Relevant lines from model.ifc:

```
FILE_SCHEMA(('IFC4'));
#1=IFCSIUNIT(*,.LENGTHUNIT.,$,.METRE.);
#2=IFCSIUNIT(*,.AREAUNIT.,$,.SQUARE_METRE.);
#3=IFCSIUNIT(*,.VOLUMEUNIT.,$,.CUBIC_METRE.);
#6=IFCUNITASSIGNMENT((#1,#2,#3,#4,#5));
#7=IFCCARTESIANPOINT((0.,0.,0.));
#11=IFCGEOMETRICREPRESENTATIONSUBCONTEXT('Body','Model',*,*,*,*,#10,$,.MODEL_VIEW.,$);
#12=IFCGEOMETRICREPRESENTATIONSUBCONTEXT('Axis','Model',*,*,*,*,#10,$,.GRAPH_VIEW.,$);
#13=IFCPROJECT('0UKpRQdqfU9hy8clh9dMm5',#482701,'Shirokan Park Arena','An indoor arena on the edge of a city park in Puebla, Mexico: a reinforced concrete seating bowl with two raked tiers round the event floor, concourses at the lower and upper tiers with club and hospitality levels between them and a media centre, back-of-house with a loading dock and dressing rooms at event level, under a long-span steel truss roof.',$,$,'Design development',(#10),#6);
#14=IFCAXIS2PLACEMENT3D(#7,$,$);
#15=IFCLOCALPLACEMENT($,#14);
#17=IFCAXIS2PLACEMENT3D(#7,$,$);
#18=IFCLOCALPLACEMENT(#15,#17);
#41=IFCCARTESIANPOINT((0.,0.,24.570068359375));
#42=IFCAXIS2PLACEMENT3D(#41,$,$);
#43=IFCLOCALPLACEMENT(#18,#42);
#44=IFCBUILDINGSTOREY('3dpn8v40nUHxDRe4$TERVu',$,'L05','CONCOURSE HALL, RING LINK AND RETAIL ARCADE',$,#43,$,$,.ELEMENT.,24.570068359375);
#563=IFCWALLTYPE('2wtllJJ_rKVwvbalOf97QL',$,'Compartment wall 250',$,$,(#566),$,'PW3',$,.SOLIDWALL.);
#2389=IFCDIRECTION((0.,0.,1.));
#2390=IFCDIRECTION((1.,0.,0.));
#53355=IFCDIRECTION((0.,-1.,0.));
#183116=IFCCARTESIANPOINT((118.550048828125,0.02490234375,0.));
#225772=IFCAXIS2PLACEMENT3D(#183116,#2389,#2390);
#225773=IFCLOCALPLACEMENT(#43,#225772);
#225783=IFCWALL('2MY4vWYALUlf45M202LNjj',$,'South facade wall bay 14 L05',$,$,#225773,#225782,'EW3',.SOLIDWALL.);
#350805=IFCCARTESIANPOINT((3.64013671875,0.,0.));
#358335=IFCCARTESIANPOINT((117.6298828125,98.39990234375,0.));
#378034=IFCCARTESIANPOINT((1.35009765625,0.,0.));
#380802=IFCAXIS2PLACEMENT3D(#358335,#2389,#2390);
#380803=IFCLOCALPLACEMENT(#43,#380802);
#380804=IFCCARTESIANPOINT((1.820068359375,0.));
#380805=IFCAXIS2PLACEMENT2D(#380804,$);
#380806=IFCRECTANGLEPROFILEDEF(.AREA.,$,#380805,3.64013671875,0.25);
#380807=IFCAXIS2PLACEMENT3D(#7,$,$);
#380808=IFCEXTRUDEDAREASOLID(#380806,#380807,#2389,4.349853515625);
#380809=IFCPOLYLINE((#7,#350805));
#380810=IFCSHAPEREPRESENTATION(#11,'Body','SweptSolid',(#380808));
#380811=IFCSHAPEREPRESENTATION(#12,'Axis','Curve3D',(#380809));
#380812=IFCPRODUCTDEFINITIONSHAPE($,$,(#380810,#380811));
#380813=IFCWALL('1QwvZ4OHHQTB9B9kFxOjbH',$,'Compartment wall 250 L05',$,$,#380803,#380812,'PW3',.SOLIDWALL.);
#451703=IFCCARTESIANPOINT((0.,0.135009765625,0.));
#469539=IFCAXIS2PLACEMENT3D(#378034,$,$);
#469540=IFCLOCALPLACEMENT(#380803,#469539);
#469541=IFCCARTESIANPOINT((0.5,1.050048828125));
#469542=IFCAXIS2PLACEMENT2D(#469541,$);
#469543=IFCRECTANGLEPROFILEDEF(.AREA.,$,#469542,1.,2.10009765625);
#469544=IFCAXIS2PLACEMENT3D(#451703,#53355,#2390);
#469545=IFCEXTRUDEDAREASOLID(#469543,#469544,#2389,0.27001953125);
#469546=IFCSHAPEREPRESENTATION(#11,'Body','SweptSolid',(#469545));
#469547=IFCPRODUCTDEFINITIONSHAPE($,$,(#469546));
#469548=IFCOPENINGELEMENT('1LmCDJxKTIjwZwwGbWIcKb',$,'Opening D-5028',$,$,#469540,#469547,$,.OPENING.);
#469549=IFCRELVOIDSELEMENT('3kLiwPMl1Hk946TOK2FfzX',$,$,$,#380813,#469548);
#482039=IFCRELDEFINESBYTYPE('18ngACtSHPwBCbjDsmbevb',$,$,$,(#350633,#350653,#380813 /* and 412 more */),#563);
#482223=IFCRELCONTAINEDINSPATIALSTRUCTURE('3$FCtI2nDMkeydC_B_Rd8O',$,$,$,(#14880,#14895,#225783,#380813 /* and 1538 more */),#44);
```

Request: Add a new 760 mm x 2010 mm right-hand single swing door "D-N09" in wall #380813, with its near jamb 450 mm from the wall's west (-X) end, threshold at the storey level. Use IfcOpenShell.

```python
import numpy as np
import ifcopenshell
import ifcopenshell.api.feature
import ifcopenshell.api.geometry
import ifcopenshell.api.root
import ifcopenshell.api.spatial
import ifcopenshell.geom
import ifcopenshell.util.element
import ifcopenshell.util.placement
import ifcopenshell.util.representation
import ifcopenshell.util.shape
import ifcopenshell.util.unit

model = ifcopenshell.open("model.ifc")
unit_scale = ifcopenshell.util.unit.calculate_unit_scale(model)
settings = ifcopenshell.geom.settings()


def volume(element):
    """Net volume in cubic metres, openings subtracted."""
    shape = ifcopenshell.geom.create_shape(settings, element)
    return ifcopenshell.util.shape.get_volume(shape.geometry)


wall = model.by_id(380813)
storey = ifcopenshell.util.element.get_container(wall, ifc_class="IfcBuildingStorey")
context = ifcopenshell.util.representation.get_context(model, "Model", "Body", "MODEL_VIEW")
before = volume(wall)

width, height, from_end, sill = 0.76, 2.01, 0.45, 0.0  # metres

# The wall runs along its own X axis, and the end named is its -X end.
wall_shape = ifcopenshell.geom.create_shape(settings, wall)
x, y, z = ifcopenshell.util.shape.get_vertices(wall_shape.geometry).T
start = x.min() + from_end
face, thickness = float(y.min()), float(y.max() - y.min())
wall_matrix = ifcopenshell.util.placement.get_local_placement(wall.ObjectPlacement)
level = ifcopenshell.util.placement.get_local_placement(storey.ObjectPlacement)[2, 3]


def in_wall(x, y):
    """Placement at x, y metres in the wall's axes, at sill height."""
    matrix = wall_matrix.copy()
    matrix[:, 3] = wall_matrix @ np.array([x / unit_scale, y / unit_scale, 0.0, 1.0])
    matrix[2, 3] = level + sill / unit_scale
    return matrix


# Opening: a box that overshoots both wall faces by 50 mm.
opening = ifcopenshell.api.root.create_entity(model, ifc_class="IfcOpeningElement", predefined_type="OPENING")
box = ifcopenshell.api.geometry.add_wall_representation(
    model, context=context, length=width, height=height, thickness=thickness + 0.1
)
ifcopenshell.api.geometry.assign_representation(model, product=opening, representation=box)
ifcopenshell.api.geometry.edit_object_placement(model, product=opening, matrix=in_wall(start, face - 0.05), is_si=False)
ifcopenshell.api.feature.add_feature(model, feature=opening, element=wall)

door = ifcopenshell.api.root.create_entity(model, ifc_class="IfcDoor", name="D-N09", predefined_type="DOOR")
door.OverallWidth, door.OverallHeight = width / unit_scale, height / unit_scale
door.OperationType = "SINGLE_SWING_RIGHT"
body = ifcopenshell.api.geometry.add_door_representation(
    model,
    context=context,
    overall_width=door.OverallWidth,
    overall_height=door.OverallHeight,
    operation_type="SINGLE_SWING_RIGHT",
    lining_properties={"LiningDepth": thickness / unit_scale, "ThresholdDepth": thickness / unit_scale},
)
ifcopenshell.api.geometry.assign_representation(model, product=door, representation=body)
ifcopenshell.api.spatial.assign_container(model, products=[door], relating_structure=storey)
ifcopenshell.api.feature.add_filling(model, opening=opening, element=door)

# The lining spans the wall, so the door starts at the wall face.
ifcopenshell.api.geometry.edit_object_placement(model, product=door, matrix=in_wall(start, face), is_si=False)

after = volume(wall)

print(f"wall volume {before:.3f} -> {after:.3f} m3")

model.write("model_rev.ifc")
```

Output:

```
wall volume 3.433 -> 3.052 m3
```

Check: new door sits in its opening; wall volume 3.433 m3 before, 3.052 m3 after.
